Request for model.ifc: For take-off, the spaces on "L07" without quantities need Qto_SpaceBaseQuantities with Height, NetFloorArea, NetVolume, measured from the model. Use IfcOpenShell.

First a look at what the model holds.

```python
import ifcopenshell
import ifcopenshell.util.element
import ifcopenshell.util.unit

model = ifcopenshell.open("model.ifc")
print(model.schema)
for unit_type in ("LENGTHUNIT", "AREAUNIT", "VOLUMEUNIT"):
    print(unit_type, ifcopenshell.util.unit.calculate_unit_scale(model, unit_type))
storey = next(s for s in model.by_type("IfcBuildingStorey") if s.Name == "L07")
spaces = [e for e in ifcopenshell.util.element.get_decomposition(storey) if e.is_a("IfcSpace")]
for e in sorted(spaces, key=lambda e: e.id()):
    print(e.id(), e.is_a(), e.Name, list(ifcopenshell.util.element.get_psets(e, qtos_only=True)), sep=" | ")
```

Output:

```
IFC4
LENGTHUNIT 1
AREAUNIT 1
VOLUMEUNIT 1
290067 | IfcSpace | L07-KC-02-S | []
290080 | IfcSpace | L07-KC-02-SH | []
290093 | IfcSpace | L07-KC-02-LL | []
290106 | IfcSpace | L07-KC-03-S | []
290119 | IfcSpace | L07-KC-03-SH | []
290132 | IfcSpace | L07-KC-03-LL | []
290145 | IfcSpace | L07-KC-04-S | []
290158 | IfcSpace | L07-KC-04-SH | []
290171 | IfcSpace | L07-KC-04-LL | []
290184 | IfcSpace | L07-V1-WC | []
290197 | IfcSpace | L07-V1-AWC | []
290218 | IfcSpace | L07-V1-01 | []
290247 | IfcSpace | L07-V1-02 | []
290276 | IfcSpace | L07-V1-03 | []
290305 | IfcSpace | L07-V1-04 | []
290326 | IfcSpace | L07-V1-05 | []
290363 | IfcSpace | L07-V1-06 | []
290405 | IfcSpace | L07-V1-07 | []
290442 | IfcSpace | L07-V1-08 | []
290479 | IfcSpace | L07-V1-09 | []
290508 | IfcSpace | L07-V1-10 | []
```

```python
import ifcopenshell
import ifcopenshell.api.pset
import ifcopenshell.geom
import ifcopenshell.util.element
import ifcopenshell.util.shape
import ifcopenshell.util.unit

model = ifcopenshell.open("model.ifc")
unit_scale = ifcopenshell.util.unit.calculate_unit_scale(model)
area_scale = ifcopenshell.util.unit.calculate_unit_scale(model, "AREAUNIT")
volume_scale = ifcopenshell.util.unit.calculate_unit_scale(model, "VOLUMEUNIT")
settings = ifcopenshell.geom.settings()

storey = next(s for s in model.by_type("IfcBuildingStorey") if s.Name == "L07")
spaces = [e for e in ifcopenshell.util.element.get_decomposition(storey) if e.is_a("IfcSpace")]

for e in sorted(spaces, key=lambda e: e.id()):
    if ifcopenshell.util.element.get_psets(e, qtos_only=True, should_inherit=False):
        continue
    # Geometry comes back in metres, in the element's own axes.
    shape = ifcopenshell.geom.create_shape(settings, e)
    values = {
        "Height": ifcopenshell.util.shape.get_z(shape.geometry) / unit_scale,
        "NetFloorArea": ifcopenshell.util.shape.get_footprint_area(shape.geometry) / area_scale,
        "NetVolume": ifcopenshell.util.shape.get_volume(shape.geometry) / volume_scale,
    }
    qto = ifcopenshell.api.pset.add_qto(model, product=e, name="Qto_SpaceBaseQuantities")
    ifcopenshell.api.pset.edit_qto(model, qto=qto, properties=values)
    print(e.id(), {k: round(v, 3) for k, v in values.items()})

model.write("model_v2.ifc")
```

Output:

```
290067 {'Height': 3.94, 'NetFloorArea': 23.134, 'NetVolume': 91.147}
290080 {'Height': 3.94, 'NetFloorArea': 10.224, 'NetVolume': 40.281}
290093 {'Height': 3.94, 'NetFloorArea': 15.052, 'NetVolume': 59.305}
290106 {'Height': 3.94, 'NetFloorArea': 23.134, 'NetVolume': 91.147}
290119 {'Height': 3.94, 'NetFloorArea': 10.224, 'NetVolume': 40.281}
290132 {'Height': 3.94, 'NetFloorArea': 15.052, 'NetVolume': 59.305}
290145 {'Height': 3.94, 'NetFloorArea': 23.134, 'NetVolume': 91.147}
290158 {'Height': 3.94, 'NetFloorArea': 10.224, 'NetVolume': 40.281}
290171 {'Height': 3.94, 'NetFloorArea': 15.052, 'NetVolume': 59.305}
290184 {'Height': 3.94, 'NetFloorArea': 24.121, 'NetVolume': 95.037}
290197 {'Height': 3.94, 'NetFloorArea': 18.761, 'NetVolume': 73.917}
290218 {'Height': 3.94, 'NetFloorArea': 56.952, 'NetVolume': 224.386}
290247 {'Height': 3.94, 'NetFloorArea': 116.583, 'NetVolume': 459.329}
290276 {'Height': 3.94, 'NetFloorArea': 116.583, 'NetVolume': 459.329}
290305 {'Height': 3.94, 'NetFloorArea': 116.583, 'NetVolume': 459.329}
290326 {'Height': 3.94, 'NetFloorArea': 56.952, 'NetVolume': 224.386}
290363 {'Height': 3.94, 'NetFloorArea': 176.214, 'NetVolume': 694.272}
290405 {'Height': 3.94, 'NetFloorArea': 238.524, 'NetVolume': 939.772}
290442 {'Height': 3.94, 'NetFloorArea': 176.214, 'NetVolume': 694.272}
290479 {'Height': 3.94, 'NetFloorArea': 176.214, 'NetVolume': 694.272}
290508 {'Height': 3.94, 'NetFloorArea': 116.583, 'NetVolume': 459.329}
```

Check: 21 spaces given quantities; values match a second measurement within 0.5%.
